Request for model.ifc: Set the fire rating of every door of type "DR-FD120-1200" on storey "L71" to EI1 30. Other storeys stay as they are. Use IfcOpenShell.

First a look at what the model holds.

```python
import ifcopenshell
import ifcopenshell.util.element

model = ifcopenshell.open("model.ifc")
print(model.schema)
storey = next(s for s in model.by_type("IfcBuildingStorey") if s.Name == "L71")
doors = [e for e in ifcopenshell.util.element.get_decomposition(storey) if e.is_a("IfcDoor")]
seen = {}
for e in doors:
    element_type = ifcopenshell.util.element.get_type(e)
    key = (element_type.Name if element_type != e and element_type else None, ifcopenshell.util.element.get_pset(e, "Pset_DoorCommon", "FireRating"))
    seen[key] = seen.get(key, 0) + 1
for (name, value), count in sorted(seen.items(), key=str):
    print(count, "x", name, "|", value)
```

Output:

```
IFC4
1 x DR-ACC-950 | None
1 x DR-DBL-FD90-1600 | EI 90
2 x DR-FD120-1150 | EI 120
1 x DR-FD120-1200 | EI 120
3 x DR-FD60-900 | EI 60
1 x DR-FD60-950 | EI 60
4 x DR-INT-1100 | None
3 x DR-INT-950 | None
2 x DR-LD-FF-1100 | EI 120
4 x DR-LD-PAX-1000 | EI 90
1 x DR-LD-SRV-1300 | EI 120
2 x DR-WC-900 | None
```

```python
import ifcopenshell
import ifcopenshell.api.pset
import ifcopenshell.util.element

model = ifcopenshell.open("model.ifc")

storey = next(s for s in model.by_type("IfcBuildingStorey") if s.Name == "L71")
doors = [e for e in ifcopenshell.util.element.get_decomposition(storey) if e.is_a("IfcDoor")]

count = 0
for e in doors:
    element_type = ifcopenshell.util.element.get_type(e)
    if element_type in (None, e) or element_type.Name != "DR-FD120-1200":
        continue
    found = ifcopenshell.util.element.get_pset(e, "Pset_DoorCommon", should_inherit=False)
    if found:
        pset = model.by_id(found["id"])
        if len(ifcopenshell.util.element.get_elements_by_pset(pset)) > 1:
            pset = ifcopenshell.api.pset.unshare_pset(model, products=[e], pset=pset)[0]
    else:
        pset = ifcopenshell.api.pset.add_pset(model, product=e, name="Pset_DoorCommon")
    ifcopenshell.api.pset.edit_pset(model, pset=pset, properties={"FireRating": "EI1 30"})
    count += 1

print(count, "doors updated")

model.write("model-out.ifc")
```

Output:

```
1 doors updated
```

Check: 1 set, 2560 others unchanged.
